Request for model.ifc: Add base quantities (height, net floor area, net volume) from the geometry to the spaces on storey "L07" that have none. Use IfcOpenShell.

First a look at what the model holds.

```python
import ifcopenshell
import ifcopenshell.util.element
import ifcopenshell.util.unit

model = ifcopenshell.open("model.ifc")
print(model.schema)
for unit_type in ("LENGTHUNIT", "AREAUNIT", "VOLUMEUNIT"):
    print(unit_type, ifcopenshell.util.unit.calculate_unit_scale(model, unit_type))
storey = next(s for s in model.by_type("IfcBuildingStorey") if s.Name == "L07")
spaces = [e for e in ifcopenshell.util.element.get_decomposition(storey) if e.is_a("IfcSpace")]
for e in sorted(spaces, key=lambda e: e.id()):
    print(e.id(), e.is_a(), e.Name, list(ifcopenshell.util.element.get_psets(e, qtos_only=True)), sep=" | ")
```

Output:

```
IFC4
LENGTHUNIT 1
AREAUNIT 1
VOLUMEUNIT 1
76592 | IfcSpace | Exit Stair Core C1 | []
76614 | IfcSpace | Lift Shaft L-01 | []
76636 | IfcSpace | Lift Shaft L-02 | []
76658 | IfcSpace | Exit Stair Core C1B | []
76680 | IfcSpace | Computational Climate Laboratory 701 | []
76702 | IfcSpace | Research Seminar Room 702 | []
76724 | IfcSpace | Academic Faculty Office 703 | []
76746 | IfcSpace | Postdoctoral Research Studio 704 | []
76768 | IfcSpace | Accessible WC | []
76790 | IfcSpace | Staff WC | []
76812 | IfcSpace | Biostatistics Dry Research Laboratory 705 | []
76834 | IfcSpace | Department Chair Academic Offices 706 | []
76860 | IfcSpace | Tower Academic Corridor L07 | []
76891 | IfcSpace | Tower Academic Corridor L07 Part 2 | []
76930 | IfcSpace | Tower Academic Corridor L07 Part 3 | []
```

```python
import ifcopenshell
import ifcopenshell.api.pset
import ifcopenshell.geom
import ifcopenshell.util.element
import ifcopenshell.util.shape
import ifcopenshell.util.unit

model = ifcopenshell.open("model.ifc")
unit_scale = ifcopenshell.util.unit.calculate_unit_scale(model)
area_scale = ifcopenshell.util.unit.calculate_unit_scale(model, "AREAUNIT")
volume_scale = ifcopenshell.util.unit.calculate_unit_scale(model, "VOLUMEUNIT")
settings = ifcopenshell.geom.settings()

storey = next(s for s in model.by_type("IfcBuildingStorey") if s.Name == "L07")
spaces = [e for e in ifcopenshell.util.element.get_decomposition(storey) if e.is_a("IfcSpace")]

for e in sorted(spaces, key=lambda e: e.id()):
    if ifcopenshell.util.element.get_psets(e, qtos_only=True, should_inherit=False):
        continue
    # Geometry comes back in metres, in the element's own axes.
    shape = ifcopenshell.geom.create_shape(settings, e)
    values = {
        "Height": ifcopenshell.util.shape.get_z(shape.geometry) / unit_scale,
        "NetFloorArea": ifcopenshell.util.shape.get_footprint_area(shape.geometry) / area_scale,
        "NetVolume": ifcopenshell.util.shape.get_volume(shape.geometry) / volume_scale,
    }
    qto = ifcopenshell.api.pset.add_qto(model, product=e, name="Qto_SpaceBaseQuantities")
    ifcopenshell.api.pset.edit_qto(model, qto=qto, properties=values)
    print(e.id(), {k: round(v, 3) for k, v in values.items()})

model.write("model_edited.ifc")
```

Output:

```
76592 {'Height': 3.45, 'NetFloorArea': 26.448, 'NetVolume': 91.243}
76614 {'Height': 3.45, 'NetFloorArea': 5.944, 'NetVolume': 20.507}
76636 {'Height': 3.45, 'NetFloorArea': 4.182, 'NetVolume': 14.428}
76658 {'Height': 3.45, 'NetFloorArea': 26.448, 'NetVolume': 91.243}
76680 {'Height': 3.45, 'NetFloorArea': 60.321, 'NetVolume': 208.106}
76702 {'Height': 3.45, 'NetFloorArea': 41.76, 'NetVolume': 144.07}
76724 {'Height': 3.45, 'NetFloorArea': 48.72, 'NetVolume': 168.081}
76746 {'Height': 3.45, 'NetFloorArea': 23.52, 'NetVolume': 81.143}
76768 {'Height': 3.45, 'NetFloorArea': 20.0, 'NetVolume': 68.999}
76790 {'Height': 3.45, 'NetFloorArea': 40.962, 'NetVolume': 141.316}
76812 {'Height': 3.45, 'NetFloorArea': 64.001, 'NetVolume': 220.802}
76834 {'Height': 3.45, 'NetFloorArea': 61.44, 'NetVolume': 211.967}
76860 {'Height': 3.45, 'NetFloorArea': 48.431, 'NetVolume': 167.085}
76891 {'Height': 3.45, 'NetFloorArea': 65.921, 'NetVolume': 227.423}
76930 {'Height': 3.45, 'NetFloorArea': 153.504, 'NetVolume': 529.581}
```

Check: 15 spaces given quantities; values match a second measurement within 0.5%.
